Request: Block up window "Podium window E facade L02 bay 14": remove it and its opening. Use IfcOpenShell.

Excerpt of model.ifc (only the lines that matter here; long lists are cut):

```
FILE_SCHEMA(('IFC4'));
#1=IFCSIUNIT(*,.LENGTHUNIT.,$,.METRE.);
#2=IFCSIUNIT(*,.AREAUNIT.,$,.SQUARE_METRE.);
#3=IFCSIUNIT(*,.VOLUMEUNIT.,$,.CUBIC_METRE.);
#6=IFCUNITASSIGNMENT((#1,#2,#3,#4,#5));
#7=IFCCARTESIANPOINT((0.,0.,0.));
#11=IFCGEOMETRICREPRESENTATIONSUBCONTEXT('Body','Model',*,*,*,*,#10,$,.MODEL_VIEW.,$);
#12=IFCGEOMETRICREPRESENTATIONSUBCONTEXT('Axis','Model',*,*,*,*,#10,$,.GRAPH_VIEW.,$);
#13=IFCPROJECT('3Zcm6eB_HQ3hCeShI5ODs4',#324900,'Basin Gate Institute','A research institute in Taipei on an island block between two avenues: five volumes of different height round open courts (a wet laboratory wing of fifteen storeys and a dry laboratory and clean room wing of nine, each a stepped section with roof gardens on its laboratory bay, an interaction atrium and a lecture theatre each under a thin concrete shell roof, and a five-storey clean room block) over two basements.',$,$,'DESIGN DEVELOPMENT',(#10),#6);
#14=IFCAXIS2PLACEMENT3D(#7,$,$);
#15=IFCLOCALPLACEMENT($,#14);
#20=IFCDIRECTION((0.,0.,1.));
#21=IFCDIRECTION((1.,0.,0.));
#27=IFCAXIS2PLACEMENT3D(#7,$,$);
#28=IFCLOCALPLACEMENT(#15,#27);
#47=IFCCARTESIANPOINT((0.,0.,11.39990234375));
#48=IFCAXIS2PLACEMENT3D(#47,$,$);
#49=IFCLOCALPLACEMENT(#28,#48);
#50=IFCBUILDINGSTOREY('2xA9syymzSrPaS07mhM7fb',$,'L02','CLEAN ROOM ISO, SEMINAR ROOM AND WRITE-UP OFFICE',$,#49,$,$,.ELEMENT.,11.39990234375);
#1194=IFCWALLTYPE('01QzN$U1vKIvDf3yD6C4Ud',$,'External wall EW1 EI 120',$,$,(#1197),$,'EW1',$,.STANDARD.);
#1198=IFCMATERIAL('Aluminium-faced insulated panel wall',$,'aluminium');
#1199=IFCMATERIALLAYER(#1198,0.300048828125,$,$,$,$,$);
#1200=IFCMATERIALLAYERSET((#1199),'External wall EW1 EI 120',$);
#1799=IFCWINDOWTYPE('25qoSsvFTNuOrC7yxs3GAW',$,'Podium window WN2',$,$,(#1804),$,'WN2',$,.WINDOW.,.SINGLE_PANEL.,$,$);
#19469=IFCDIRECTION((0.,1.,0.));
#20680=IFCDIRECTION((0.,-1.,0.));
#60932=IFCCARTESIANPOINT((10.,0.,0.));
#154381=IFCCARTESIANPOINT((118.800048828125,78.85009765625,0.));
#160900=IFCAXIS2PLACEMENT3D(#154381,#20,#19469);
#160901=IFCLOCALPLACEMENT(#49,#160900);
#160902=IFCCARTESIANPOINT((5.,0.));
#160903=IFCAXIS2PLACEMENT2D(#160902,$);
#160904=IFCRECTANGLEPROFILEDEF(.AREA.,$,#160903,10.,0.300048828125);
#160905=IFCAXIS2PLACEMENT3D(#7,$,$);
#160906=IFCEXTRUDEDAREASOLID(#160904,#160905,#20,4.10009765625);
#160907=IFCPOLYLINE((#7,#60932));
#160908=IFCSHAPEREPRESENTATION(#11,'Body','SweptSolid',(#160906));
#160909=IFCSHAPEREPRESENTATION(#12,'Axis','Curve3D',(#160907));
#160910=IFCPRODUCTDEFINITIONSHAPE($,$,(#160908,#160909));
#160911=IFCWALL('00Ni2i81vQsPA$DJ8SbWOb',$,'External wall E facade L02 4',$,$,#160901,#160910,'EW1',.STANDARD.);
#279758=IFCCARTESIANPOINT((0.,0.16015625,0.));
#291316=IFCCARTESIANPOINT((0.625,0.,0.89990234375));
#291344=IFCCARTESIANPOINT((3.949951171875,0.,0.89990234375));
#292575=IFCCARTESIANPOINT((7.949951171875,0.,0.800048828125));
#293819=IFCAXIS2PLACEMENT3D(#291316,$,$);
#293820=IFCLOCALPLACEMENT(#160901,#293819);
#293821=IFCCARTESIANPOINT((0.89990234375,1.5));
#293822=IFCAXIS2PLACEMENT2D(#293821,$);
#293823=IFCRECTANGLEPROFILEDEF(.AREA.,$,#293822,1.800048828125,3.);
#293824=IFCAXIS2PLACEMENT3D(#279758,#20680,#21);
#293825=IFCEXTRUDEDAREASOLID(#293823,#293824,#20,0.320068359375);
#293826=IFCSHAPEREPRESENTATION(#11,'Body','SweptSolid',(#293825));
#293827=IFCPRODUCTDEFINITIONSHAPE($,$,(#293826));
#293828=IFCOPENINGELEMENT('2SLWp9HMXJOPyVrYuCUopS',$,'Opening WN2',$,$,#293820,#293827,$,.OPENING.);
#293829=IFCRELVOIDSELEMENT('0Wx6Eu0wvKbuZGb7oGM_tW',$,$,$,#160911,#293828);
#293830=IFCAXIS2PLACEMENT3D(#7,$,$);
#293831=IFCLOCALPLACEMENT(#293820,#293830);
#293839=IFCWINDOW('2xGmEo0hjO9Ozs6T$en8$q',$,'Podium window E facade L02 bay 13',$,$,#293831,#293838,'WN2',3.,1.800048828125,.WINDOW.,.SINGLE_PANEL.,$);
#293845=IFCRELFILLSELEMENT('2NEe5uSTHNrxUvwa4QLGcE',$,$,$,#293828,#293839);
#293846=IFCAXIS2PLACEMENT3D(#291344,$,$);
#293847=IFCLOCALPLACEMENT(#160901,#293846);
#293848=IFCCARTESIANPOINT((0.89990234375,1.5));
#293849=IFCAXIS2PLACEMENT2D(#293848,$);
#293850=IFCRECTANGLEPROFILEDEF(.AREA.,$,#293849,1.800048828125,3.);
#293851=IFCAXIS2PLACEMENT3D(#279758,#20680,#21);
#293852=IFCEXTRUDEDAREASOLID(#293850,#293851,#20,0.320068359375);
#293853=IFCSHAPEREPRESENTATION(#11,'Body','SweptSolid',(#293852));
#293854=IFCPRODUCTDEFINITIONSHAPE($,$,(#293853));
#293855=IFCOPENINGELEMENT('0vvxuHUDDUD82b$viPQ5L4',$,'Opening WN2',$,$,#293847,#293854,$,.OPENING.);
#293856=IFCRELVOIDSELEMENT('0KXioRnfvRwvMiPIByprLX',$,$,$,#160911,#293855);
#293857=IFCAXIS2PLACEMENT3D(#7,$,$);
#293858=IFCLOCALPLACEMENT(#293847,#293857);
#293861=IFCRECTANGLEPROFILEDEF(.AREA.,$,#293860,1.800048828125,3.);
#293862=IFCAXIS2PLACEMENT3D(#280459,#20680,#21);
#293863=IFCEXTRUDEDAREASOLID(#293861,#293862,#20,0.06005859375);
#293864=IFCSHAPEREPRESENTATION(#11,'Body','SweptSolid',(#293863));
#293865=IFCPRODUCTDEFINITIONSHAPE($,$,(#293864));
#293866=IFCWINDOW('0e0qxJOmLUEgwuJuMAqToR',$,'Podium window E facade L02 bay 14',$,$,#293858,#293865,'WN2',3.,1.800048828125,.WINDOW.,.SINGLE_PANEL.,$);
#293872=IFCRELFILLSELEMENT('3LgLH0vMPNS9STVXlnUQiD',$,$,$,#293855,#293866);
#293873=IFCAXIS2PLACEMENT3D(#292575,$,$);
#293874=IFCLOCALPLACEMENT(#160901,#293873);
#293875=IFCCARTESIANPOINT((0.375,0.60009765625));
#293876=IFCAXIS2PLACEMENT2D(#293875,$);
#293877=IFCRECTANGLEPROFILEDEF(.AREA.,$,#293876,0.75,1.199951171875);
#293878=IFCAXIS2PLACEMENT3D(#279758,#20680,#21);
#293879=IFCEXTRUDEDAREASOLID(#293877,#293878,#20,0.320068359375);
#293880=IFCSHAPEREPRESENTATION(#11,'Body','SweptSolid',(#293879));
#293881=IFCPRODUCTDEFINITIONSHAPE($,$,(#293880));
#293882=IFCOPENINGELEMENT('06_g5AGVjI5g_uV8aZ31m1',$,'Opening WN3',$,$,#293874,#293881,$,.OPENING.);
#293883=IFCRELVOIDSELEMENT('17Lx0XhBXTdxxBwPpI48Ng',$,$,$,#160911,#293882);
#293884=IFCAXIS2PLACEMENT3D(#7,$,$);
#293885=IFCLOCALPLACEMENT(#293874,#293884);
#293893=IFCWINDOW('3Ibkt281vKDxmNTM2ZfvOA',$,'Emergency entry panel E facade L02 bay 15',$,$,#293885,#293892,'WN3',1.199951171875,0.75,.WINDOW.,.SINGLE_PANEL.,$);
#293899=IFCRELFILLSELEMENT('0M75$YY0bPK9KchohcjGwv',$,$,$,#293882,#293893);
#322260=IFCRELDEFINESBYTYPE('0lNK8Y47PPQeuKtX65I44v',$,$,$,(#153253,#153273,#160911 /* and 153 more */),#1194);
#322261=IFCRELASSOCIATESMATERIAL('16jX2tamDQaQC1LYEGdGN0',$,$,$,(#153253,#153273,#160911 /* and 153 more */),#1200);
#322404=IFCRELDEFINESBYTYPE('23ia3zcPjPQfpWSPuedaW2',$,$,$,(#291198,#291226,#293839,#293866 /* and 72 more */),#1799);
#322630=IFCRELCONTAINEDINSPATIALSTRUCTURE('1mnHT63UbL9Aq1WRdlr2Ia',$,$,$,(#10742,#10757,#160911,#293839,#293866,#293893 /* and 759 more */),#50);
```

```python
import ifcopenshell
import ifcopenshell.api.feature
import ifcopenshell.api.root
import ifcopenshell.geom
import ifcopenshell.util.shape

model = ifcopenshell.open("model.ifc")
settings = ifcopenshell.geom.settings()


def volume(element):
    """Net volume in cubic metres, openings subtracted."""
    shape = ifcopenshell.geom.create_shape(settings, element)
    return ifcopenshell.util.shape.get_volume(shape.geometry)


window = model.by_guid("0e0qxJOmLUEgwuJuMAqToR")
opening = window.FillsVoids[0].RelatingOpeningElement
wall = opening.VoidsElements[0].RelatingBuildingElement
before = volume(wall)

ifcopenshell.api.root.remove_product(model, product=window)
ifcopenshell.api.feature.remove_feature(model, feature=opening)

after = volume(wall)

print(f"wall volume {before:.3f} -> {after:.3f} m3")

model.write("model_edited.ifc")
```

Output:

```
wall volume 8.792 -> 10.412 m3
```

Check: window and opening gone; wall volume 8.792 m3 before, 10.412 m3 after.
